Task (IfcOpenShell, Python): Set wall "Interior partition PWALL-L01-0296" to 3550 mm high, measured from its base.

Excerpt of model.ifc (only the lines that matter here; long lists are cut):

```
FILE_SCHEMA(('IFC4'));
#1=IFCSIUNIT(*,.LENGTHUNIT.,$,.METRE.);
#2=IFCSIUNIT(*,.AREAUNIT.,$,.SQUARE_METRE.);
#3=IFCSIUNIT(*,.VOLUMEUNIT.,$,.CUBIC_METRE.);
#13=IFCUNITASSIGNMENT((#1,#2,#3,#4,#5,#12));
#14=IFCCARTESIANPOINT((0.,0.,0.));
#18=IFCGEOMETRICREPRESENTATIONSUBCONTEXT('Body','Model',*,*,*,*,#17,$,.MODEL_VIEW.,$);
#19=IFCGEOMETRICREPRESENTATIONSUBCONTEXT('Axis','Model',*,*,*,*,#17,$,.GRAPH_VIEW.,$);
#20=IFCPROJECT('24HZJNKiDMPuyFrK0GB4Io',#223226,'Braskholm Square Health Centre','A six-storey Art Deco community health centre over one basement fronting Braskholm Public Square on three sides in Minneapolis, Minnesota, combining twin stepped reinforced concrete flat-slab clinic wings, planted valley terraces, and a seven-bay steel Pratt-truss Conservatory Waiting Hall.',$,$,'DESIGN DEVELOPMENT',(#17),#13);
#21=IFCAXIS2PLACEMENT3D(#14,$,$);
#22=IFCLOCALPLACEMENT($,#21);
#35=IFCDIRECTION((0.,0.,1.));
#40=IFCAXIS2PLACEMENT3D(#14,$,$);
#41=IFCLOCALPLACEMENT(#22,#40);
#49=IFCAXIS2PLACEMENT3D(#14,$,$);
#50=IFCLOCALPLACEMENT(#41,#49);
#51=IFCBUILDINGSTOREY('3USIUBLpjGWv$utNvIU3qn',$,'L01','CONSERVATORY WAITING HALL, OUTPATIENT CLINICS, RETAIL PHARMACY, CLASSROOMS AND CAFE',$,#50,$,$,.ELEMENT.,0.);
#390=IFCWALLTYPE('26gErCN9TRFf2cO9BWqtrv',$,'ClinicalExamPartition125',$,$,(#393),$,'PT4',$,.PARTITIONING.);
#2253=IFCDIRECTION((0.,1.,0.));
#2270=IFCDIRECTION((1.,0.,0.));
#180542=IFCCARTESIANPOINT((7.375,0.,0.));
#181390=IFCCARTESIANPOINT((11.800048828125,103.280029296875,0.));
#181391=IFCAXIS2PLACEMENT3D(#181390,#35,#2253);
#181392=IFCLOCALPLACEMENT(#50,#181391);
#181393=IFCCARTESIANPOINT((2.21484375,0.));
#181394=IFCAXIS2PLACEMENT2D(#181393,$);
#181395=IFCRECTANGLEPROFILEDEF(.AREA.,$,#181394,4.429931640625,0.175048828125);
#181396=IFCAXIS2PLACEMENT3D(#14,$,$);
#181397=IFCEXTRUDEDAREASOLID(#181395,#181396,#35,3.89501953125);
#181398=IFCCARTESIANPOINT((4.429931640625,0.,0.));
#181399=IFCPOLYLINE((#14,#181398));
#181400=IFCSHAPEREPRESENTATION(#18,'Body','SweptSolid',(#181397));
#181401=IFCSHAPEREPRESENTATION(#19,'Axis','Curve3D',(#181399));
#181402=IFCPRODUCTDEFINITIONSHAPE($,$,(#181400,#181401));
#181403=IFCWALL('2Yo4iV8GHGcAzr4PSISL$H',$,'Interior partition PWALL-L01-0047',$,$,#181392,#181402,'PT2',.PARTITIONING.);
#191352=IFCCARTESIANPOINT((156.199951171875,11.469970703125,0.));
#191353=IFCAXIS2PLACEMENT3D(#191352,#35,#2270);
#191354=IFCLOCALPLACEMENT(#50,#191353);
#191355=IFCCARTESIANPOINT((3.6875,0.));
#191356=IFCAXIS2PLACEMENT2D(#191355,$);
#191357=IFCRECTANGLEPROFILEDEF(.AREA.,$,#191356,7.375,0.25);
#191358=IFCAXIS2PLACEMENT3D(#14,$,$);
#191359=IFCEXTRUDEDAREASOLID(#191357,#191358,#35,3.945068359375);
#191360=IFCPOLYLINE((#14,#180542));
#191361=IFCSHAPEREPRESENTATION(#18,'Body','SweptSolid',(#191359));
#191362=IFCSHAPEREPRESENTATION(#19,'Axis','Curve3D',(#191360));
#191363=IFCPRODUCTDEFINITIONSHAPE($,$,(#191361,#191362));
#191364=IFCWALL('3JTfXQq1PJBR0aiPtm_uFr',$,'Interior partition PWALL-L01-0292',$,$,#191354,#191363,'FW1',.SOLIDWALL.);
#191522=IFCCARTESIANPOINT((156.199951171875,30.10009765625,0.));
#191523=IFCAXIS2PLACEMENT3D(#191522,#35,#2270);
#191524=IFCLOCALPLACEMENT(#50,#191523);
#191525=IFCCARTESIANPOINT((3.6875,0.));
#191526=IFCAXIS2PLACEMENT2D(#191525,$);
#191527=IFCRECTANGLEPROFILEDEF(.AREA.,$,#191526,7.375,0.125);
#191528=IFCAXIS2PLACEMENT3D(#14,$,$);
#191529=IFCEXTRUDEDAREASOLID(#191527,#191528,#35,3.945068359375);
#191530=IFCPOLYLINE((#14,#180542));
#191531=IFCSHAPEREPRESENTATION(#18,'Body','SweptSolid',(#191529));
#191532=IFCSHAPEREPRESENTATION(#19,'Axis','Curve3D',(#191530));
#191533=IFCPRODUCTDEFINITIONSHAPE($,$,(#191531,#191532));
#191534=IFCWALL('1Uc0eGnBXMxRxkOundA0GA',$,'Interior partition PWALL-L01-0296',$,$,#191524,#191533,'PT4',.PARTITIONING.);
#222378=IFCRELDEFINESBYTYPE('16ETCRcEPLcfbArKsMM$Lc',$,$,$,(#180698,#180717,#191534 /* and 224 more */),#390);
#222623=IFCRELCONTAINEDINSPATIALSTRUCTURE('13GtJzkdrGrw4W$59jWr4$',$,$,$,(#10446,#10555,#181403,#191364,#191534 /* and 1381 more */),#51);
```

```python
import ifcopenshell
import ifcopenshell.geom
import ifcopenshell.util.representation
import ifcopenshell.util.shape

model = ifcopenshell.open("model.ifc")
settings = ifcopenshell.geom.settings()


def volume(element):
    """Net volume in cubic metres, openings subtracted."""
    shape = ifcopenshell.geom.create_shape(settings, element)
    return ifcopenshell.util.shape.get_volume(shape.geometry)


wall = model.by_id(191534)
before = volume(wall)

body = ifcopenshell.util.representation.get_representation(wall, "Model", "Body")
solid = body.Items[0]
old_height = solid.Depth
solid.Depth = 3.55
after = volume(wall)

print(f"height {old_height:g} -> {solid.Depth:g}, volume {before:.3f} -> {after:.3f} m3")

model.write("model_rev.ifc")
```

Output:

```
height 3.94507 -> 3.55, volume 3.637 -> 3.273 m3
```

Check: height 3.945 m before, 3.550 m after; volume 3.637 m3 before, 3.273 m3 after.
